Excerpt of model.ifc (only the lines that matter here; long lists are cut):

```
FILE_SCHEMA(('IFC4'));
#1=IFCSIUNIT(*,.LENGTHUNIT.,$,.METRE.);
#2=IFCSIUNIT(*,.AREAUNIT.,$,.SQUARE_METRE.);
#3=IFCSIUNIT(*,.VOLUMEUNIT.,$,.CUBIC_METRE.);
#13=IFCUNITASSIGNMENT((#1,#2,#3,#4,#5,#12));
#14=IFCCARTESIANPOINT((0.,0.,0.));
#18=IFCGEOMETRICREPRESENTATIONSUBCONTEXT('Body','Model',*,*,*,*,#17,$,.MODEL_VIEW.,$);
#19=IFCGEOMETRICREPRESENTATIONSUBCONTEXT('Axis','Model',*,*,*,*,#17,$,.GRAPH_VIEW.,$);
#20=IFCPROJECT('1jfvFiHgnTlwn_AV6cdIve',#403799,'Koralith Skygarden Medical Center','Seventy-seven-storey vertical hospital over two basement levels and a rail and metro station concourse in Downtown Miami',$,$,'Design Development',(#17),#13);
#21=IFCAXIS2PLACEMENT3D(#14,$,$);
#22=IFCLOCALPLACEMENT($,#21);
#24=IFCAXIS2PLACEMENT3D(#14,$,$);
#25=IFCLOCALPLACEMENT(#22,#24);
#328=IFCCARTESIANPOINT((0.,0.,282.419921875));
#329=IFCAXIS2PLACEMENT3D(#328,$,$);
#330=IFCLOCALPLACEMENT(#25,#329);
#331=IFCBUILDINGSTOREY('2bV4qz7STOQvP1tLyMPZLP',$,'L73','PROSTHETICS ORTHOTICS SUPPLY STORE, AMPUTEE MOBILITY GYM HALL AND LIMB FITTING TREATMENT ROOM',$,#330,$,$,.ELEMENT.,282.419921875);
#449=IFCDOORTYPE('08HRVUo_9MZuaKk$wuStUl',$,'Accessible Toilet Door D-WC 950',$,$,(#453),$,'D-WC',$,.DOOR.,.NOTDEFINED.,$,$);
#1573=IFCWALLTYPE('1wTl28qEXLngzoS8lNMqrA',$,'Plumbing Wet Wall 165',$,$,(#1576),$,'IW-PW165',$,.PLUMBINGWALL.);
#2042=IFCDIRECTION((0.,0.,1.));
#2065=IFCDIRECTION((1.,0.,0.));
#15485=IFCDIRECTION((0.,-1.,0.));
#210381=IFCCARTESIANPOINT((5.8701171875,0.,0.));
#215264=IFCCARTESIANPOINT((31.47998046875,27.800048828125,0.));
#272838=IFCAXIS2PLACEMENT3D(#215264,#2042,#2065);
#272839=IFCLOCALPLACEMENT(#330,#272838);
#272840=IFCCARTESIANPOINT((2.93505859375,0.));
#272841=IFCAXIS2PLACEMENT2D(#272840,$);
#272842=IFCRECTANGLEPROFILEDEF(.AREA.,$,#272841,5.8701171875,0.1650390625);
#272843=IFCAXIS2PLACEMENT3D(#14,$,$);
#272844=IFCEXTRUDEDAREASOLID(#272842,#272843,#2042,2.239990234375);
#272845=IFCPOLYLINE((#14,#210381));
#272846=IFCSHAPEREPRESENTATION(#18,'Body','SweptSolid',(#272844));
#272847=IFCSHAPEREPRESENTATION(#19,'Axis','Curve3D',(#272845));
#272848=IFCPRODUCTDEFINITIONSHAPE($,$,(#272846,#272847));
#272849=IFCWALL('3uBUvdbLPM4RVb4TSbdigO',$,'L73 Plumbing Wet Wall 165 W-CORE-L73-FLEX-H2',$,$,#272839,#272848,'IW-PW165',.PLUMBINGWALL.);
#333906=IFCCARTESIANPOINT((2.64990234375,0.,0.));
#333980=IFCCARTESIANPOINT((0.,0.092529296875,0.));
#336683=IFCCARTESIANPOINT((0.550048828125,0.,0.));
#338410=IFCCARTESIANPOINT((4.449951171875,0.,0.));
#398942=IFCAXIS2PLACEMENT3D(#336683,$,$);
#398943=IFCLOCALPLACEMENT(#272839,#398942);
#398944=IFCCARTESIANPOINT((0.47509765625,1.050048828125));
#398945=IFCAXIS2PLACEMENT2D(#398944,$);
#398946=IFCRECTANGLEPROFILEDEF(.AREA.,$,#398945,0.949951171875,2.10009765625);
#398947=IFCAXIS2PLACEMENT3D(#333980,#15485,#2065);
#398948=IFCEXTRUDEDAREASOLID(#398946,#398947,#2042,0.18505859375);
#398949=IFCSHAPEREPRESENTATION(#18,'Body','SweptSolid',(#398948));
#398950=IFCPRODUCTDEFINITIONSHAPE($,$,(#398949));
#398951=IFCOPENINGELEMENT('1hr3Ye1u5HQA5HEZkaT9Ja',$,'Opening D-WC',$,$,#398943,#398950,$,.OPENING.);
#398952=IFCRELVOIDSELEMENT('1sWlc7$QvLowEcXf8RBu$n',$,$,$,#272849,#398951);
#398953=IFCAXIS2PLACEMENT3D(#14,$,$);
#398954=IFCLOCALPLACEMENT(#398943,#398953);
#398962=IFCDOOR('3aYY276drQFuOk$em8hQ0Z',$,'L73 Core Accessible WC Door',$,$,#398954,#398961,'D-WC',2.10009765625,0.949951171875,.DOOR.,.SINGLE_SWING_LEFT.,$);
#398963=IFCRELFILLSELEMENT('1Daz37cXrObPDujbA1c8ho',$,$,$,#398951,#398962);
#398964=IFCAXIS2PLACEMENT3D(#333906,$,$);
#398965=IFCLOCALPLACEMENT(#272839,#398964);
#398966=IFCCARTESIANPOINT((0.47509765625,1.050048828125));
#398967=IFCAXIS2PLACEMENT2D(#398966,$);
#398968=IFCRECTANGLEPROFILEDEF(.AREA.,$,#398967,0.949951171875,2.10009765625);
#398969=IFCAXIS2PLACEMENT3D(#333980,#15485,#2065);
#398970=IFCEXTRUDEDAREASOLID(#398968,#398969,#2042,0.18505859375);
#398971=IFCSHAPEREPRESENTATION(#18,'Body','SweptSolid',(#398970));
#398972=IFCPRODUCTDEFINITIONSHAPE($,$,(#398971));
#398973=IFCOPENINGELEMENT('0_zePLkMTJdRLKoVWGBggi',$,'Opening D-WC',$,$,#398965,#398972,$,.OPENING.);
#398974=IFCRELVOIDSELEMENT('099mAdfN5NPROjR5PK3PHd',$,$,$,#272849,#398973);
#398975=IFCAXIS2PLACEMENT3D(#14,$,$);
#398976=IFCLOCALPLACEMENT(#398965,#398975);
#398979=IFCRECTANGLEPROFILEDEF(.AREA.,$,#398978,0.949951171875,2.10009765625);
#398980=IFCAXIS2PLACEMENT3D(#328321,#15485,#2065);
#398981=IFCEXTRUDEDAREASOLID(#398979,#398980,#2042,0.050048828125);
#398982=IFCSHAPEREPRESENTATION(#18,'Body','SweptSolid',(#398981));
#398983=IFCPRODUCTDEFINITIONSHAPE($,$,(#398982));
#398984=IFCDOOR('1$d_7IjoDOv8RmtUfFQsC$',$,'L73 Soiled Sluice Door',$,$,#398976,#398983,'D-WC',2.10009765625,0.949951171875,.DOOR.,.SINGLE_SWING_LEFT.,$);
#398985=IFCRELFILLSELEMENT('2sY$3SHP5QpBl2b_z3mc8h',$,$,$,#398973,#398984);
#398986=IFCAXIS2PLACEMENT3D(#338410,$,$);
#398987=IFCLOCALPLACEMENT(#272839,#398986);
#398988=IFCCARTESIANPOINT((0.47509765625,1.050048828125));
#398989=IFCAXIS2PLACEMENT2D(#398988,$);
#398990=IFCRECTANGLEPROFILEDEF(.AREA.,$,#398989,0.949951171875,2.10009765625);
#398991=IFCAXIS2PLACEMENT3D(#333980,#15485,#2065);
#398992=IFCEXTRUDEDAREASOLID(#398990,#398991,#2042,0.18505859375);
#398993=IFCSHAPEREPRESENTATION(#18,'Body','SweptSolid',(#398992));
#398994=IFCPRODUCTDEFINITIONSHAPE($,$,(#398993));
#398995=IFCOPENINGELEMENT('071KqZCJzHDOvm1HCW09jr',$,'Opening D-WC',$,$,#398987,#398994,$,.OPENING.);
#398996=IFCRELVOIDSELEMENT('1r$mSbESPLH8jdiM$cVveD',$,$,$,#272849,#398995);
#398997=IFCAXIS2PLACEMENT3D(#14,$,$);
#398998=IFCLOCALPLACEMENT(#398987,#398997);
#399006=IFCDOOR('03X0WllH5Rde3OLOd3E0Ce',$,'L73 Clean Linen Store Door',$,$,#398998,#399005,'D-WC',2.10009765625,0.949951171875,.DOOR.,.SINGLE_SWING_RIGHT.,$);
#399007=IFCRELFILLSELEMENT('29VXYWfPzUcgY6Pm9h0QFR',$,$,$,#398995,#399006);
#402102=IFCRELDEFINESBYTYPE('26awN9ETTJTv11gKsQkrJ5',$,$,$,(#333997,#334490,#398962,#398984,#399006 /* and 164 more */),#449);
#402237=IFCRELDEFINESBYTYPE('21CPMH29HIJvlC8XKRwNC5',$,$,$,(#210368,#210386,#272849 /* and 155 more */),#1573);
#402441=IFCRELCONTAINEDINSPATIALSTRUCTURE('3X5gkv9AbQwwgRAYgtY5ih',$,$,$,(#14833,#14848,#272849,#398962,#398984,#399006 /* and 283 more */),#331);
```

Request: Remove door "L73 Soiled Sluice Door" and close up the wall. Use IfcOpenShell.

```python
import ifcopenshell
import ifcopenshell.api.feature
import ifcopenshell.api.root
import ifcopenshell.geom
import ifcopenshell.util.shape

model = ifcopenshell.open("model.ifc")
settings = ifcopenshell.geom.settings()


def volume(element):
    """Net volume in cubic metres, openings subtracted."""
    shape = ifcopenshell.geom.create_shape(settings, element)
    return ifcopenshell.util.shape.get_volume(shape.geometry)


door = model.by_id(398984)
opening = door.FillsVoids[0].RelatingOpeningElement
wall = opening.VoidsElements[0].RelatingBuildingElement
before = volume(wall)

ifcopenshell.api.root.remove_product(model, product=door)
ifcopenshell.api.feature.remove_feature(model, feature=opening)

after = volume(wall)

print(f"wall volume {before:.3f} -> {after:.3f} m3")

model.write("model_edited.ifc")
```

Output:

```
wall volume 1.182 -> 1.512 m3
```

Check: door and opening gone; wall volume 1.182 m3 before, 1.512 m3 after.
